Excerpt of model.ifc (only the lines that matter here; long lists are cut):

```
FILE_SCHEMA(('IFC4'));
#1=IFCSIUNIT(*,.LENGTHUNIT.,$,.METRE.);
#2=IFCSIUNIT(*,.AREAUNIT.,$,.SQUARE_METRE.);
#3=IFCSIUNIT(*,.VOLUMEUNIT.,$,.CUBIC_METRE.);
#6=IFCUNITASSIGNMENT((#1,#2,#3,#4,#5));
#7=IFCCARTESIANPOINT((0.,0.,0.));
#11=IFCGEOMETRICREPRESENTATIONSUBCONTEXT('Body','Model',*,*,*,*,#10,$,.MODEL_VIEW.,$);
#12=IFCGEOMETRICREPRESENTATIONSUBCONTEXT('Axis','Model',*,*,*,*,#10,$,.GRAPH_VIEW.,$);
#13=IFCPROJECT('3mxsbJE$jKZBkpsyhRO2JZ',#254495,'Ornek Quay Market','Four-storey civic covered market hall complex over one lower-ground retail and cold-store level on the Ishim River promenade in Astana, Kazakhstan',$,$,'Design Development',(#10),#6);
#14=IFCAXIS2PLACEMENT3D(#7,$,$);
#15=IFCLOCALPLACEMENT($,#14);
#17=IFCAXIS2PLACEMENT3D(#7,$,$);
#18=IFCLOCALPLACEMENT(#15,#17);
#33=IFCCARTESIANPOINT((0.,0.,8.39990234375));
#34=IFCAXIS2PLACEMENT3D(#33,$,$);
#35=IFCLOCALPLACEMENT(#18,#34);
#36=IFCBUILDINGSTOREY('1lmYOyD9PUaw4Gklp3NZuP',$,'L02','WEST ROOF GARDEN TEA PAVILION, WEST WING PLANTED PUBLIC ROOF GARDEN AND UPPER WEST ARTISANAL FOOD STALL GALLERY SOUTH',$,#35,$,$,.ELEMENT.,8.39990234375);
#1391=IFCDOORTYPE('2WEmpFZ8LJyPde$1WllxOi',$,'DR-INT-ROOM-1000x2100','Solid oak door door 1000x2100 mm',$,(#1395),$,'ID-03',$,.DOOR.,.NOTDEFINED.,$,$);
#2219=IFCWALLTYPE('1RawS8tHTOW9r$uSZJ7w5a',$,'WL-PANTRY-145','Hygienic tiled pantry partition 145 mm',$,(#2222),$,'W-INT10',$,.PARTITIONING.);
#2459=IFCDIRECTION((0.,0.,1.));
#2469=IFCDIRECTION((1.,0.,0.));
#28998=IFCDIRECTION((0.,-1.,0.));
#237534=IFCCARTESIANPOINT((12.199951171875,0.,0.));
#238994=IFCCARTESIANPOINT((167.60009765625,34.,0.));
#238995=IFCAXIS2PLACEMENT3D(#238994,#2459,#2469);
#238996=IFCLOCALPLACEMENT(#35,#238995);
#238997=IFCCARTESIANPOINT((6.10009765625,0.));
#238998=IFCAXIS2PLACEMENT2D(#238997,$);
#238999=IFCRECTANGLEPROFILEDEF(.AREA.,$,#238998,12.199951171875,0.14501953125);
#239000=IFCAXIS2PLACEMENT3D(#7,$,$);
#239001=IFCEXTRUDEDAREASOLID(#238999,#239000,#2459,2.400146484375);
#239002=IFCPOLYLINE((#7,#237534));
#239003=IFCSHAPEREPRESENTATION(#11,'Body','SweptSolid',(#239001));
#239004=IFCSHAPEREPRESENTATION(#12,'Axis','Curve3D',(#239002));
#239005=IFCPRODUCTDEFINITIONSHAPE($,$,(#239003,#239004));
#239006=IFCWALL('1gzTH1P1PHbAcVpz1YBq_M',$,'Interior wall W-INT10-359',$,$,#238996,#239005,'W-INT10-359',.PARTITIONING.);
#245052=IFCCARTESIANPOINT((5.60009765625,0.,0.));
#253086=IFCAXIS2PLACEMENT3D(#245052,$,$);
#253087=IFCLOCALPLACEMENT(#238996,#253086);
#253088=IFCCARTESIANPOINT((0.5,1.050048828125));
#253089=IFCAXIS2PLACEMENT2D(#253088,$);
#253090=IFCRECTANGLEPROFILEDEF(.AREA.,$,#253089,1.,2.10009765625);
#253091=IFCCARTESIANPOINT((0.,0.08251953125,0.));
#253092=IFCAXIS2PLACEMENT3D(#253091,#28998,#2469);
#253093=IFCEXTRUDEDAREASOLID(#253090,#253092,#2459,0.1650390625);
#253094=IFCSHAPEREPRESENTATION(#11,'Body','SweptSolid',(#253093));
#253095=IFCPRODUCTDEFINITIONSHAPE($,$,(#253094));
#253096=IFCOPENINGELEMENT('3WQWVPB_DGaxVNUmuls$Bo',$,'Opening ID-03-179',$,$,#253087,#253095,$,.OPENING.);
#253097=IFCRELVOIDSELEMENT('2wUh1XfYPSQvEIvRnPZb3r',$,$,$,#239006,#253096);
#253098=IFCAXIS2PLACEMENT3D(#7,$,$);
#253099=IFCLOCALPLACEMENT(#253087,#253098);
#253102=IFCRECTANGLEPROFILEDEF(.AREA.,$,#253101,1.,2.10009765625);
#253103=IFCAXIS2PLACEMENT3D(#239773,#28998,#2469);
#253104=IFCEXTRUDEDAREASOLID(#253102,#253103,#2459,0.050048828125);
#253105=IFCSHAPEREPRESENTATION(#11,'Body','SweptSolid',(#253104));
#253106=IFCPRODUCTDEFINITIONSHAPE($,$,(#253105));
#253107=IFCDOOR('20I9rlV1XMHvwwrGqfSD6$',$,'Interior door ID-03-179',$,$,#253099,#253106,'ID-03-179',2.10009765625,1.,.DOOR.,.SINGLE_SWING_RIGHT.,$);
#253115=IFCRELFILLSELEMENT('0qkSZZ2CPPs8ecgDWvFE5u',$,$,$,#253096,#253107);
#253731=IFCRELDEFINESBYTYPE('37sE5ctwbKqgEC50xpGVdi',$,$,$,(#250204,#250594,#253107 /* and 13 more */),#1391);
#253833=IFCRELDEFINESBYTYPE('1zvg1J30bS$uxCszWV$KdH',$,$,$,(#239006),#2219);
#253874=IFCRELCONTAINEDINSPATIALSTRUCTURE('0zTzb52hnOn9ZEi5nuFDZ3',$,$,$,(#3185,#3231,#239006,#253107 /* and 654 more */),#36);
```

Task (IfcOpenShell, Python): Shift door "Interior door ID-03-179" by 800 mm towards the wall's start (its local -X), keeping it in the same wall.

```python
import ifcopenshell
import ifcopenshell.api.geometry
import ifcopenshell.util.placement
import ifcopenshell.util.unit

model = ifcopenshell.open("model.ifc")
unit_scale = ifcopenshell.util.unit.calculate_unit_scale(model)

door = model.by_id(253107)
opening = door.FillsVoids[0].RelatingOpeningElement
wall = opening.VoidsElements[0].RelatingBuildingElement

wall_matrix = ifcopenshell.util.placement.get_local_placement(wall.ObjectPlacement)
shift = wall_matrix[:3, 0] * -0.8 / unit_scale
before = ifcopenshell.util.placement.get_local_placement(door.ObjectPlacement)[:3, 3].copy()

# The door is placed relative to its opening, so it follows when the opening moves.
matrix = ifcopenshell.util.placement.get_local_placement(opening.ObjectPlacement)
matrix[:3, 3] += shift
ifcopenshell.api.geometry.edit_object_placement(
    model, product=opening, matrix=matrix, is_si=False, should_transform_children=True
)

after = ifcopenshell.util.placement.get_local_placement(door.ObjectPlacement)[:3, 3]
print("door moved by", (after - before).round(3) + 0.0)

model.write("model_updated.ifc")
```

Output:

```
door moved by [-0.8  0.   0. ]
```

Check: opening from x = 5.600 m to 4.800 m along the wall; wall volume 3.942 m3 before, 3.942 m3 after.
